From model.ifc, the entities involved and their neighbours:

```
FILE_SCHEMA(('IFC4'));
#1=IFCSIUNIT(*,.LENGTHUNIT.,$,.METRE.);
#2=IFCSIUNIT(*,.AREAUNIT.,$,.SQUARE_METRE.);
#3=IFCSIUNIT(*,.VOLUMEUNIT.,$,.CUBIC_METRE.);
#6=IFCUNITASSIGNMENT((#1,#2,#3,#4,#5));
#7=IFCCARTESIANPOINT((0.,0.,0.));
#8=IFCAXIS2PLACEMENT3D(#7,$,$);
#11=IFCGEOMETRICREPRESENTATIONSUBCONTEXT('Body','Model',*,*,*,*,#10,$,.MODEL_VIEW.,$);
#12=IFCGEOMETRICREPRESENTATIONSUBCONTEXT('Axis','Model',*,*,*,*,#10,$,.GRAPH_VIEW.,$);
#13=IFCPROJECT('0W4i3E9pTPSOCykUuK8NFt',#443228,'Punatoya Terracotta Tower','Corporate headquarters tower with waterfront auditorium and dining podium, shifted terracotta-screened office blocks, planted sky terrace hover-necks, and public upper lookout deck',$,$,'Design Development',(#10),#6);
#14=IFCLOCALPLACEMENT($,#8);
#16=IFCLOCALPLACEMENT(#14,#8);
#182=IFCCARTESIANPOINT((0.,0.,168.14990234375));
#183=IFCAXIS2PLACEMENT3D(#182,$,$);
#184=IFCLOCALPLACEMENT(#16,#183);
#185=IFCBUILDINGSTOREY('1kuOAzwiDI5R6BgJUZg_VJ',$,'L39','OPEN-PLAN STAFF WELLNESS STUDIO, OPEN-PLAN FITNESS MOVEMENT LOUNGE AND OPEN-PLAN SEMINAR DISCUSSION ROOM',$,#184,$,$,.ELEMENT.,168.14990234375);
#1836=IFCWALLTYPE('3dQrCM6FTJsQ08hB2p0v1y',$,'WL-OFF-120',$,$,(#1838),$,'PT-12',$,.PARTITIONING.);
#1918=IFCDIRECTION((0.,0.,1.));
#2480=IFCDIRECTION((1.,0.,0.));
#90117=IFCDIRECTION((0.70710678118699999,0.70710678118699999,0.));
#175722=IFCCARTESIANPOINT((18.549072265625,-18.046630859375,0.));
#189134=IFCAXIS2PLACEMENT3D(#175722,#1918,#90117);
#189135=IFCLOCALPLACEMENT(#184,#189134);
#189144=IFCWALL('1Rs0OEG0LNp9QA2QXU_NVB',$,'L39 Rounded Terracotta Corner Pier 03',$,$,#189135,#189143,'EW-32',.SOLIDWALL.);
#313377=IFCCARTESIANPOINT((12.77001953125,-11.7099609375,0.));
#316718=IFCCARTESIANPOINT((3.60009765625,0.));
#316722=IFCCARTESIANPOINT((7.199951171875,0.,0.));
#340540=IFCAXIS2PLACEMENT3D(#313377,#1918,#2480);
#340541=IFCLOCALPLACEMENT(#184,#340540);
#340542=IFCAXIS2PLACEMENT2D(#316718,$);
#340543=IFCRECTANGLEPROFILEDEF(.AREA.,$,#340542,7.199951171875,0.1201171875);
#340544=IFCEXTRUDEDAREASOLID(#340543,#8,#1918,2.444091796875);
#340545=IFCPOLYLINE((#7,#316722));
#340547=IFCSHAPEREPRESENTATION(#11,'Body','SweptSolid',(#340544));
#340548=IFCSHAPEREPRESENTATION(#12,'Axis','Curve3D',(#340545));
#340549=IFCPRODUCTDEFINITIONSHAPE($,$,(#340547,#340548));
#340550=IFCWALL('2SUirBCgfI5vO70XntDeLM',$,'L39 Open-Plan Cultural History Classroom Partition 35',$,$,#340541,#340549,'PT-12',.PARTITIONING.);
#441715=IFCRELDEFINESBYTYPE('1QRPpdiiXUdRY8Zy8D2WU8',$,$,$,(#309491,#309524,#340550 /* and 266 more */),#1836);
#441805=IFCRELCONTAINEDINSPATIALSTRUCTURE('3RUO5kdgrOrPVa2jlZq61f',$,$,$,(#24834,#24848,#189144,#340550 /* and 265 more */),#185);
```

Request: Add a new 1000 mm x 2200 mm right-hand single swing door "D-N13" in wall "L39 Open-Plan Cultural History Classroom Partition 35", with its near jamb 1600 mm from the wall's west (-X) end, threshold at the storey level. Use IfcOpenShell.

```python
import numpy as np
import ifcopenshell
import ifcopenshell.api.feature
import ifcopenshell.api.geometry
import ifcopenshell.api.root
import ifcopenshell.api.spatial
import ifcopenshell.geom
import ifcopenshell.util.element
import ifcopenshell.util.placement
import ifcopenshell.util.representation
import ifcopenshell.util.shape
import ifcopenshell.util.unit

model = ifcopenshell.open("model.ifc")
unit_scale = ifcopenshell.util.unit.calculate_unit_scale(model)
settings = ifcopenshell.geom.settings()


def volume(element):
    """Net volume in cubic metres, openings subtracted."""
    shape = ifcopenshell.geom.create_shape(settings, element)
    return ifcopenshell.util.shape.get_volume(shape.geometry)


wall = model.by_guid("2SUirBCgfI5vO70XntDeLM")
storey = ifcopenshell.util.element.get_container(wall, ifc_class="IfcBuildingStorey")
context = ifcopenshell.util.representation.get_context(model, "Model", "Body", "MODEL_VIEW")
before = volume(wall)

width, height, from_end, sill = 1, 2.2, 1.6, 0.0  # metres

# The wall runs along its own X axis, and the end named is its -X end.
wall_shape = ifcopenshell.geom.create_shape(settings, wall)
x, y, z = ifcopenshell.util.shape.get_vertices(wall_shape.geometry).T
start = x.min() + from_end
face, thickness = float(y.min()), float(y.max() - y.min())
wall_matrix = ifcopenshell.util.placement.get_local_placement(wall.ObjectPlacement)
level = ifcopenshell.util.placement.get_local_placement(storey.ObjectPlacement)[2, 3]


def in_wall(x, y):
    """Placement at x, y metres in the wall's axes, at sill height."""
    matrix = wall_matrix.copy()
    matrix[:, 3] = wall_matrix @ np.array([x / unit_scale, y / unit_scale, 0.0, 1.0])
    matrix[2, 3] = level + sill / unit_scale
    return matrix


# Opening: a box that overshoots both wall faces by 50 mm.
opening = ifcopenshell.api.root.create_entity(model, ifc_class="IfcOpeningElement", predefined_type="OPENING")
box = ifcopenshell.api.geometry.add_wall_representation(
    model, context=context, length=width, height=height, thickness=thickness + 0.1
)
ifcopenshell.api.geometry.assign_representation(model, product=opening, representation=box)
ifcopenshell.api.geometry.edit_object_placement(model, product=opening, matrix=in_wall(start, face - 0.05), is_si=False)
ifcopenshell.api.feature.add_feature(model, feature=opening, element=wall)

door = ifcopenshell.api.root.create_entity(model, ifc_class="IfcDoor", name="D-N13", predefined_type="DOOR")
door.OverallWidth, door.OverallHeight = width / unit_scale, height / unit_scale
door.OperationType = "SINGLE_SWING_RIGHT"
body = ifcopenshell.api.geometry.add_door_representation(
    model,
    context=context,
    overall_width=door.OverallWidth,
    overall_height=door.OverallHeight,
    operation_type="SINGLE_SWING_RIGHT",
    lining_properties={"LiningDepth": thickness / unit_scale, "ThresholdDepth": thickness / unit_scale},
)
ifcopenshell.api.geometry.assign_representation(model, product=door, representation=body)
ifcopenshell.api.spatial.assign_container(model, products=[door], relating_structure=storey)
ifcopenshell.api.feature.add_filling(model, opening=opening, element=door)

# The lining spans the wall, so the door starts at the wall face.
ifcopenshell.api.geometry.edit_object_placement(model, product=door, matrix=in_wall(start, face), is_si=False)

after = volume(wall)

print(f"wall volume {before:.3f} -> {after:.3f} m3")

model.write("model_v2.ifc")
```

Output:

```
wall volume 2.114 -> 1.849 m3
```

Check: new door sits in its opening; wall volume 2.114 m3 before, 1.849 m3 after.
